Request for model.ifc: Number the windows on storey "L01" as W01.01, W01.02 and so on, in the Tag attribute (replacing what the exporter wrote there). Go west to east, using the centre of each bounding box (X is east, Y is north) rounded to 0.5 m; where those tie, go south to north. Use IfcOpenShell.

First a look at what the model holds.

```python
import ifcopenshell
import ifcopenshell.util.element
import ifcopenshell.util.placement

model = ifcopenshell.open("model.ifc")
print(model.schema)
storey = next(s for s in model.by_type("IfcBuildingStorey") if s.Name == "L01")
windows = [e for e in ifcopenshell.util.element.get_decomposition(storey) if e.is_a("IfcWindow")]
for e in sorted(windows, key=lambda e: e.id()):
    origin = ifcopenshell.util.placement.get_local_placement(e.ObjectPlacement)[:3, 3]
    print(e.id(), e.Tag, e.Name, origin.round(2) + 0.0, sep=" | ")
```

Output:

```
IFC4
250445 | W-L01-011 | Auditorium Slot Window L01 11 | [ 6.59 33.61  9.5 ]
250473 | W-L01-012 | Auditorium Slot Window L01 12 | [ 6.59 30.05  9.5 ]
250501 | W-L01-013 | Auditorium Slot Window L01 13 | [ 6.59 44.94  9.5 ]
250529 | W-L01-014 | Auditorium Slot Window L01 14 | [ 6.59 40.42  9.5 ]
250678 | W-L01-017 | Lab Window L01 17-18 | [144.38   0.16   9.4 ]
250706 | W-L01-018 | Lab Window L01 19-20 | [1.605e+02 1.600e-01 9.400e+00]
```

```python
import ifcopenshell
import ifcopenshell.geom
import ifcopenshell.util.element
import ifcopenshell.util.shape

model = ifcopenshell.open("model.ifc")
settings = ifcopenshell.geom.settings()
settings.set("use-world-coords", True)


def centre(element):
    shape = ifcopenshell.geom.create_shape(settings, element)
    return ifcopenshell.util.shape.get_bbox_centroid(shape.geometry)


storey = next(s for s in model.by_type("IfcBuildingStorey") if s.Name == "L01")
windows = [e for e in ifcopenshell.util.element.get_decomposition(storey) if e.is_a("IfcWindow")]

# Insertion points can sit at a corner or the storey origin, so sort by the geometry (in metres).
centres = {e: centre(e) for e in windows}
windows.sort(key=lambda e: (round(centres[e][0] / 0.5), centres[e][1]))

for i, e in enumerate(windows, start=1):
    number = f"W01.{i:02d}"
    e.Tag = number
    print(e.id(), number)

model.write("model-out.ifc")
```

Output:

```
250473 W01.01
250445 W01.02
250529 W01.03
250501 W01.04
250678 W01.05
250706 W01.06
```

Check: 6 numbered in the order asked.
